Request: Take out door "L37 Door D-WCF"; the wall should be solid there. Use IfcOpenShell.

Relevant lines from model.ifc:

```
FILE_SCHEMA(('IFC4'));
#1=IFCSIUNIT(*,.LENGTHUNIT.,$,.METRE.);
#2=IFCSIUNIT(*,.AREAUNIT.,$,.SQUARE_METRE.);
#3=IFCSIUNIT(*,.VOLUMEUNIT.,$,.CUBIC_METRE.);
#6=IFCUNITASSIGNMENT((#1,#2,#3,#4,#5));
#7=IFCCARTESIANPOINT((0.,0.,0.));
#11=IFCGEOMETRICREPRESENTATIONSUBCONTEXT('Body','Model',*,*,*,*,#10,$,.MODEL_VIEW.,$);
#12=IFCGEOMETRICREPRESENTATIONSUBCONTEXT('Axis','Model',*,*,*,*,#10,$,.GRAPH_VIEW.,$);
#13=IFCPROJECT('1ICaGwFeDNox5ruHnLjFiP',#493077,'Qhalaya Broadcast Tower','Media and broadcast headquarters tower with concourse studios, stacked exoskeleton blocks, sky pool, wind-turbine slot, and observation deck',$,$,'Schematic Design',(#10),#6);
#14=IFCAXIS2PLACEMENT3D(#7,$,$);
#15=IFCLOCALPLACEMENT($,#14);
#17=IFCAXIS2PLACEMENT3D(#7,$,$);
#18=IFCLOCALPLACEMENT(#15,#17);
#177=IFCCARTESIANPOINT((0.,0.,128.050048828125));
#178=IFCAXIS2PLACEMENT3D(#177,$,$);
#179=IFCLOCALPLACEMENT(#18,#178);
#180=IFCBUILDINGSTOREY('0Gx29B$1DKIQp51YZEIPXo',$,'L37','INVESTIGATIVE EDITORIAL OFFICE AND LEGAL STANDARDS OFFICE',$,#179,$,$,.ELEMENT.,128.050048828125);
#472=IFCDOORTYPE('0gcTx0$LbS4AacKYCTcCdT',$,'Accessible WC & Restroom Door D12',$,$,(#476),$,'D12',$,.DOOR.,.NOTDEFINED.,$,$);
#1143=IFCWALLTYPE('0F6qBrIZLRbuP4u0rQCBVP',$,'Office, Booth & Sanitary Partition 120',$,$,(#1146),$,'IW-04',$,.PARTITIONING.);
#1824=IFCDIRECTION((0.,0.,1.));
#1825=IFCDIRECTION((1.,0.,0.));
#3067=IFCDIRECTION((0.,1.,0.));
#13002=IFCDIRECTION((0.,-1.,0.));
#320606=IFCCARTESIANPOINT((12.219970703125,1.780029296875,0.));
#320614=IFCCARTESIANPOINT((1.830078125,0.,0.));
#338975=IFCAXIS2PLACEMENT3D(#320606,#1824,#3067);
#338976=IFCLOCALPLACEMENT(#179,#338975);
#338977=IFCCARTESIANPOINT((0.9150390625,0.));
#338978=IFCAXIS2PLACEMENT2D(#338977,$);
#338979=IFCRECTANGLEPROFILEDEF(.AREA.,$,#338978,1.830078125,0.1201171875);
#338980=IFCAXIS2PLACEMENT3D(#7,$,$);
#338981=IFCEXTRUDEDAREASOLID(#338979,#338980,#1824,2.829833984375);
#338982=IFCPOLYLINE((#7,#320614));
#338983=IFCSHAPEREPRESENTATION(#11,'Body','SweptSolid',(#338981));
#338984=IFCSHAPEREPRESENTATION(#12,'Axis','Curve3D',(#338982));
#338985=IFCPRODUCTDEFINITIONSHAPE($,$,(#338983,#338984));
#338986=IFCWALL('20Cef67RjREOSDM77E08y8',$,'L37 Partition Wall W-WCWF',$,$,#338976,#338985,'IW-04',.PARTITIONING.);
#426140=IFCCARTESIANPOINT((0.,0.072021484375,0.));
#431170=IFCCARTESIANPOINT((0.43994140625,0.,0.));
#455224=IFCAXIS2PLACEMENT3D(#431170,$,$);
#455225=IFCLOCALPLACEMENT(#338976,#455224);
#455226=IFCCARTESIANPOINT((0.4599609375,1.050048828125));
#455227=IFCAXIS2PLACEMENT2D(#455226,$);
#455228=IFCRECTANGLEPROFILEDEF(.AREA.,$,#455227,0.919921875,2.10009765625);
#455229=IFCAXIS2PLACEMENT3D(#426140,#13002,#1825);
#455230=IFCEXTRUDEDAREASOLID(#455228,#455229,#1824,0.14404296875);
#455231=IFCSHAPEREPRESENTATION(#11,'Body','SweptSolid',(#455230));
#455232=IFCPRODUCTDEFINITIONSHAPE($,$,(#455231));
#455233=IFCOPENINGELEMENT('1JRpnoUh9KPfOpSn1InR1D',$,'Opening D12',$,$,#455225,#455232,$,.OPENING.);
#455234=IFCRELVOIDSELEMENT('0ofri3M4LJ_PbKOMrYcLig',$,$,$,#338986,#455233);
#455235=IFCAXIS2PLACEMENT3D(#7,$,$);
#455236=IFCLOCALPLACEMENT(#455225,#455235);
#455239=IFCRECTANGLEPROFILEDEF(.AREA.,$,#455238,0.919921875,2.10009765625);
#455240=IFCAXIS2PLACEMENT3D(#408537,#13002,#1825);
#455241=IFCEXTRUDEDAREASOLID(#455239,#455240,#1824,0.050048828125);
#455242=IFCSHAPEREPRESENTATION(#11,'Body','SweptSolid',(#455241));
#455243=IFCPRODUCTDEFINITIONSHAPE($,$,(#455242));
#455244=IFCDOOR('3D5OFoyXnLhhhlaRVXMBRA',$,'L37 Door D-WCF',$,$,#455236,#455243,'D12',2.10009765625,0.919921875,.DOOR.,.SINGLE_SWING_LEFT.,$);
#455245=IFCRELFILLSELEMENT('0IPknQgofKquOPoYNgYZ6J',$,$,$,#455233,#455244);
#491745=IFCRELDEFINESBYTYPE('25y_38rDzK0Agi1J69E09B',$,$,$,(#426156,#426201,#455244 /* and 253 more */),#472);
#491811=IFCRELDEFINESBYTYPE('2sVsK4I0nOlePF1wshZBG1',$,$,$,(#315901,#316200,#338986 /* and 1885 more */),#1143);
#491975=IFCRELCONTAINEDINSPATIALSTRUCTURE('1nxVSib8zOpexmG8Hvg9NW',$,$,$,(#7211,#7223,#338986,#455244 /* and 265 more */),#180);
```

```python
import ifcopenshell
import ifcopenshell.api.feature
import ifcopenshell.api.root
import ifcopenshell.geom
import ifcopenshell.util.shape

model = ifcopenshell.open("model.ifc")
settings = ifcopenshell.geom.settings()


def volume(element):
    """Net volume in cubic metres, openings subtracted."""
    shape = ifcopenshell.geom.create_shape(settings, element)
    return ifcopenshell.util.shape.get_volume(shape.geometry)


door = model.by_id(455244)
opening = door.FillsVoids[0].RelatingOpeningElement
wall = opening.VoidsElements[0].RelatingBuildingElement
before = volume(wall)

ifcopenshell.api.root.remove_product(model, product=door)
ifcopenshell.api.feature.remove_feature(model, feature=opening)

after = volume(wall)

print(f"wall volume {before:.3f} -> {after:.3f} m3")

model.write("model_updated.ifc")
```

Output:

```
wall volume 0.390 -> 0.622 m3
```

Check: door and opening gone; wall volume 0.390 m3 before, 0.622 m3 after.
